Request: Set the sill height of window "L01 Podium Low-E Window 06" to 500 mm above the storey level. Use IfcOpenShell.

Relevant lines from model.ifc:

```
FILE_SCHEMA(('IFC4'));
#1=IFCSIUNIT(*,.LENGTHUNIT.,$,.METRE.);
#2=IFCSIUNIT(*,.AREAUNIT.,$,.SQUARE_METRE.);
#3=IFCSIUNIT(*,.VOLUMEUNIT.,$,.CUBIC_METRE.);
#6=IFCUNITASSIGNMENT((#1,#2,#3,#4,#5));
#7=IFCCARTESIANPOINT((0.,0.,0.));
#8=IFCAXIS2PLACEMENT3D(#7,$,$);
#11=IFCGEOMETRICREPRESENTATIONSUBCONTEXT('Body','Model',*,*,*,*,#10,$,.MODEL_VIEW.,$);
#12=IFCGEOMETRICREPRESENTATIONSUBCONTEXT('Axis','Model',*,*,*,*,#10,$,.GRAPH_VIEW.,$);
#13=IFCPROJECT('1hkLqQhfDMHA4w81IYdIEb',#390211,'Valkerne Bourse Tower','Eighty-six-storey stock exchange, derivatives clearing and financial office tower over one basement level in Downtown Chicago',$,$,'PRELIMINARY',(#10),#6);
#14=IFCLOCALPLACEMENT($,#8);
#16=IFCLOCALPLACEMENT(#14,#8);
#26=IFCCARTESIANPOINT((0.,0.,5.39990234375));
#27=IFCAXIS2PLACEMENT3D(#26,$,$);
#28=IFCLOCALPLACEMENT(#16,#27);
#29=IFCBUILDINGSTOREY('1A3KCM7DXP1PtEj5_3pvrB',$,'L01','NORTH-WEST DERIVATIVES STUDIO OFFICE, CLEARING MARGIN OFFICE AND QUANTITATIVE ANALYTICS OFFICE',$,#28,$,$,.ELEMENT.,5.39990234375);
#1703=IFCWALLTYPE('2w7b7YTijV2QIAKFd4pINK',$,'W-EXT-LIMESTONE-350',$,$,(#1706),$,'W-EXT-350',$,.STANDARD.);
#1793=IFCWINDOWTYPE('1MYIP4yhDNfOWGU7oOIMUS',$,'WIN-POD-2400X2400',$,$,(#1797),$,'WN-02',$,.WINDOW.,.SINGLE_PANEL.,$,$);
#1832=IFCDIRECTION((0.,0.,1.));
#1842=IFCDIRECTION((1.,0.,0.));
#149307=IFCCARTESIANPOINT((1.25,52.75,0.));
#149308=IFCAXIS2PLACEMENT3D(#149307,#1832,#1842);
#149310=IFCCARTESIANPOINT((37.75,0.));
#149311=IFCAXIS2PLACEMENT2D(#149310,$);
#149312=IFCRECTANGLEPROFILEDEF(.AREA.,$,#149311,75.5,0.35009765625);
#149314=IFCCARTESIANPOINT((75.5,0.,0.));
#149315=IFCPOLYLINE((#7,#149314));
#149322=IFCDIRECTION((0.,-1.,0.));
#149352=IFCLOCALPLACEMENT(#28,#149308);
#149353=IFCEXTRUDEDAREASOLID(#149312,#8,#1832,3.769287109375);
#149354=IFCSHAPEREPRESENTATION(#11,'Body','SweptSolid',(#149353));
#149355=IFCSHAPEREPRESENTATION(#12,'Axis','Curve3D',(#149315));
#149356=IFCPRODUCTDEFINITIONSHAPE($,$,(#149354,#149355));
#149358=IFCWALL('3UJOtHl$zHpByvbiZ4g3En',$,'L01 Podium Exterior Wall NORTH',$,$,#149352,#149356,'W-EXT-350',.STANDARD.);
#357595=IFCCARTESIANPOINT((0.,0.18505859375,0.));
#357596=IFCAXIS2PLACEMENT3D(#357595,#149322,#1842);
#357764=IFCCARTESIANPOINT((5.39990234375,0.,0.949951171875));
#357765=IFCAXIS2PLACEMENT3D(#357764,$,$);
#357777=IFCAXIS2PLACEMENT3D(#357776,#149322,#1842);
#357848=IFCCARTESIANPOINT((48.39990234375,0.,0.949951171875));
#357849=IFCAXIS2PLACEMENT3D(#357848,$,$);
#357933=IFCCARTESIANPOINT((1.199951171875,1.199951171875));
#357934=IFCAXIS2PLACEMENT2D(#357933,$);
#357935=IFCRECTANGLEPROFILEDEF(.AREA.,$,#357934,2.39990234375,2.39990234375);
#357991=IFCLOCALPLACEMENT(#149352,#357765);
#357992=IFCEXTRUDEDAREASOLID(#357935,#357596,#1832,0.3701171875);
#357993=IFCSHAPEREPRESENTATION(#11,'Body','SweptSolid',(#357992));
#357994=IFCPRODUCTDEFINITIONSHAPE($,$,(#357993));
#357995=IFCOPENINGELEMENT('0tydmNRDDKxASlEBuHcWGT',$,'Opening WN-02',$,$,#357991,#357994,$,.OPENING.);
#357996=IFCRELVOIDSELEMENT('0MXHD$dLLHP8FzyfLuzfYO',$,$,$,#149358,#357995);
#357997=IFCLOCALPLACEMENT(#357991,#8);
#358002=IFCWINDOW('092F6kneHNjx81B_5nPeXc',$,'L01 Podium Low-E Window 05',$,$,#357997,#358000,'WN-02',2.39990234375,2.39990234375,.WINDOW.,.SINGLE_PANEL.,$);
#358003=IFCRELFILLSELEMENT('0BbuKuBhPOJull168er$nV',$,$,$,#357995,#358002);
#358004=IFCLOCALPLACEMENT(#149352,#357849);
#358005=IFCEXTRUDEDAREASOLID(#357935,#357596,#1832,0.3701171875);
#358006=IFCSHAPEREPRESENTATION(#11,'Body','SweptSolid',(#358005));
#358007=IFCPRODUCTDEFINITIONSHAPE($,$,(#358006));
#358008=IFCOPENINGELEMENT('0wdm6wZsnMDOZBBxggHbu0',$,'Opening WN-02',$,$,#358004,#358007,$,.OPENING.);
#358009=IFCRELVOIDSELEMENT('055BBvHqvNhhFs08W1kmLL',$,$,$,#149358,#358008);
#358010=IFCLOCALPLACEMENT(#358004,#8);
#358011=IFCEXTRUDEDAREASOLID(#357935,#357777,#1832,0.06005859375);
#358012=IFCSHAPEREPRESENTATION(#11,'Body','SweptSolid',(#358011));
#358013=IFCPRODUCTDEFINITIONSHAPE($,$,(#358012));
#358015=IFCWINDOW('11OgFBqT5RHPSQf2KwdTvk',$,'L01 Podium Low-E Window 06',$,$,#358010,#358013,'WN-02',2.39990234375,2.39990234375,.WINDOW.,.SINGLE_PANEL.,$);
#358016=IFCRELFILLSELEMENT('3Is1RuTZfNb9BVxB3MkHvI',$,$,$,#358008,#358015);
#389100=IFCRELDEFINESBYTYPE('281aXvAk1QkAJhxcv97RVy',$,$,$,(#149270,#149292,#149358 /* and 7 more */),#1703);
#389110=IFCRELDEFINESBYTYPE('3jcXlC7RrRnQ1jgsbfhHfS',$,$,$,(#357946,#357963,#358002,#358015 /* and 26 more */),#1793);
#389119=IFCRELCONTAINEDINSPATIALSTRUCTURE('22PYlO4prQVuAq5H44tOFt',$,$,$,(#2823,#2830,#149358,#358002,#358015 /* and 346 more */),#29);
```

```python
import numpy as np
import ifcopenshell
import ifcopenshell.api.geometry
import ifcopenshell.geom
import ifcopenshell.util.element
import ifcopenshell.util.placement
import ifcopenshell.util.shape
import ifcopenshell.util.unit

model = ifcopenshell.open("model.ifc")
unit_scale = ifcopenshell.util.unit.calculate_unit_scale(model)

window = model.by_guid("11OgFBqT5RHPSQf2KwdTvk")
opening = window.FillsVoids[0].RelatingOpeningElement
storey = ifcopenshell.util.element.get_container(window, ifc_class="IfcBuildingStorey")
level = ifcopenshell.util.placement.get_local_placement(storey.ObjectPlacement)[2, 3]

# The opening's origin need not be at the sill, so measure its lowest point.
shape = ifcopenshell.geom.create_shape(ifcopenshell.geom.settings(), opening)
bottom = ifcopenshell.util.shape.get_shape_bottom_elevation(shape, shape.geometry) / unit_scale
dz = level + 0.5 / unit_scale - bottom

shift = np.array([0.0, 0.0, dz])
# The window is placed relative to its opening, so it follows when the opening moves.
matrix = ifcopenshell.util.placement.get_local_placement(opening.ObjectPlacement)
matrix[:3, 3] += shift
ifcopenshell.api.geometry.edit_object_placement(
    model, product=opening, matrix=matrix, is_si=False, should_transform_children=True
)

print(f"moved by {dz * unit_scale:+.3f} m")

model.write("model-out.ifc")
```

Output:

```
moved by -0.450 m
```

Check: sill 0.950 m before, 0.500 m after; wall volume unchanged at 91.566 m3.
